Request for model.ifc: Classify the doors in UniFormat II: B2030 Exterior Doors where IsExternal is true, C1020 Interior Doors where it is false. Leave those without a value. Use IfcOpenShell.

First a look at what the model holds.

```python
import ifcopenshell
import ifcopenshell.util.element

model = ifcopenshell.open("model.ifc")
print(model.schema)
print("classifications:", [c.Name for c in model.by_type("IfcClassification")])
values = [ifcopenshell.util.element.get_pset(e, "Pset_DoorCommon", "IsExternal") for e in model.by_type("IfcDoor")]
for value in (True, False, None):
    print("IsExternal", value, values.count(value))
```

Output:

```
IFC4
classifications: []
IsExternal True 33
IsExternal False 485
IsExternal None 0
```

```python
import ifcopenshell
import ifcopenshell.api.classification
import ifcopenshell.util.element

model = ifcopenshell.open("model.ifc")

system = ifcopenshell.api.classification.add_classification(model, classification="UniFormat II")

doors = model.by_type("IfcDoor")
external = {e: ifcopenshell.util.element.get_pset(e, "Pset_DoorCommon", "IsExternal") for e in doors}
for flag, code, name in ((True, "B2030", "Exterior Doors"), (False, "C1020", "Interior Doors")):
    products = [e for e in doors if external[e] is flag]
    ifcopenshell.api.classification.add_reference(
        model, products=products, classification=system, identification=code, name=name
    )
    print(code, len(products))

model.write("model_updated.ifc")
```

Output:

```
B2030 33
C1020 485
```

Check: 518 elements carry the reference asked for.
